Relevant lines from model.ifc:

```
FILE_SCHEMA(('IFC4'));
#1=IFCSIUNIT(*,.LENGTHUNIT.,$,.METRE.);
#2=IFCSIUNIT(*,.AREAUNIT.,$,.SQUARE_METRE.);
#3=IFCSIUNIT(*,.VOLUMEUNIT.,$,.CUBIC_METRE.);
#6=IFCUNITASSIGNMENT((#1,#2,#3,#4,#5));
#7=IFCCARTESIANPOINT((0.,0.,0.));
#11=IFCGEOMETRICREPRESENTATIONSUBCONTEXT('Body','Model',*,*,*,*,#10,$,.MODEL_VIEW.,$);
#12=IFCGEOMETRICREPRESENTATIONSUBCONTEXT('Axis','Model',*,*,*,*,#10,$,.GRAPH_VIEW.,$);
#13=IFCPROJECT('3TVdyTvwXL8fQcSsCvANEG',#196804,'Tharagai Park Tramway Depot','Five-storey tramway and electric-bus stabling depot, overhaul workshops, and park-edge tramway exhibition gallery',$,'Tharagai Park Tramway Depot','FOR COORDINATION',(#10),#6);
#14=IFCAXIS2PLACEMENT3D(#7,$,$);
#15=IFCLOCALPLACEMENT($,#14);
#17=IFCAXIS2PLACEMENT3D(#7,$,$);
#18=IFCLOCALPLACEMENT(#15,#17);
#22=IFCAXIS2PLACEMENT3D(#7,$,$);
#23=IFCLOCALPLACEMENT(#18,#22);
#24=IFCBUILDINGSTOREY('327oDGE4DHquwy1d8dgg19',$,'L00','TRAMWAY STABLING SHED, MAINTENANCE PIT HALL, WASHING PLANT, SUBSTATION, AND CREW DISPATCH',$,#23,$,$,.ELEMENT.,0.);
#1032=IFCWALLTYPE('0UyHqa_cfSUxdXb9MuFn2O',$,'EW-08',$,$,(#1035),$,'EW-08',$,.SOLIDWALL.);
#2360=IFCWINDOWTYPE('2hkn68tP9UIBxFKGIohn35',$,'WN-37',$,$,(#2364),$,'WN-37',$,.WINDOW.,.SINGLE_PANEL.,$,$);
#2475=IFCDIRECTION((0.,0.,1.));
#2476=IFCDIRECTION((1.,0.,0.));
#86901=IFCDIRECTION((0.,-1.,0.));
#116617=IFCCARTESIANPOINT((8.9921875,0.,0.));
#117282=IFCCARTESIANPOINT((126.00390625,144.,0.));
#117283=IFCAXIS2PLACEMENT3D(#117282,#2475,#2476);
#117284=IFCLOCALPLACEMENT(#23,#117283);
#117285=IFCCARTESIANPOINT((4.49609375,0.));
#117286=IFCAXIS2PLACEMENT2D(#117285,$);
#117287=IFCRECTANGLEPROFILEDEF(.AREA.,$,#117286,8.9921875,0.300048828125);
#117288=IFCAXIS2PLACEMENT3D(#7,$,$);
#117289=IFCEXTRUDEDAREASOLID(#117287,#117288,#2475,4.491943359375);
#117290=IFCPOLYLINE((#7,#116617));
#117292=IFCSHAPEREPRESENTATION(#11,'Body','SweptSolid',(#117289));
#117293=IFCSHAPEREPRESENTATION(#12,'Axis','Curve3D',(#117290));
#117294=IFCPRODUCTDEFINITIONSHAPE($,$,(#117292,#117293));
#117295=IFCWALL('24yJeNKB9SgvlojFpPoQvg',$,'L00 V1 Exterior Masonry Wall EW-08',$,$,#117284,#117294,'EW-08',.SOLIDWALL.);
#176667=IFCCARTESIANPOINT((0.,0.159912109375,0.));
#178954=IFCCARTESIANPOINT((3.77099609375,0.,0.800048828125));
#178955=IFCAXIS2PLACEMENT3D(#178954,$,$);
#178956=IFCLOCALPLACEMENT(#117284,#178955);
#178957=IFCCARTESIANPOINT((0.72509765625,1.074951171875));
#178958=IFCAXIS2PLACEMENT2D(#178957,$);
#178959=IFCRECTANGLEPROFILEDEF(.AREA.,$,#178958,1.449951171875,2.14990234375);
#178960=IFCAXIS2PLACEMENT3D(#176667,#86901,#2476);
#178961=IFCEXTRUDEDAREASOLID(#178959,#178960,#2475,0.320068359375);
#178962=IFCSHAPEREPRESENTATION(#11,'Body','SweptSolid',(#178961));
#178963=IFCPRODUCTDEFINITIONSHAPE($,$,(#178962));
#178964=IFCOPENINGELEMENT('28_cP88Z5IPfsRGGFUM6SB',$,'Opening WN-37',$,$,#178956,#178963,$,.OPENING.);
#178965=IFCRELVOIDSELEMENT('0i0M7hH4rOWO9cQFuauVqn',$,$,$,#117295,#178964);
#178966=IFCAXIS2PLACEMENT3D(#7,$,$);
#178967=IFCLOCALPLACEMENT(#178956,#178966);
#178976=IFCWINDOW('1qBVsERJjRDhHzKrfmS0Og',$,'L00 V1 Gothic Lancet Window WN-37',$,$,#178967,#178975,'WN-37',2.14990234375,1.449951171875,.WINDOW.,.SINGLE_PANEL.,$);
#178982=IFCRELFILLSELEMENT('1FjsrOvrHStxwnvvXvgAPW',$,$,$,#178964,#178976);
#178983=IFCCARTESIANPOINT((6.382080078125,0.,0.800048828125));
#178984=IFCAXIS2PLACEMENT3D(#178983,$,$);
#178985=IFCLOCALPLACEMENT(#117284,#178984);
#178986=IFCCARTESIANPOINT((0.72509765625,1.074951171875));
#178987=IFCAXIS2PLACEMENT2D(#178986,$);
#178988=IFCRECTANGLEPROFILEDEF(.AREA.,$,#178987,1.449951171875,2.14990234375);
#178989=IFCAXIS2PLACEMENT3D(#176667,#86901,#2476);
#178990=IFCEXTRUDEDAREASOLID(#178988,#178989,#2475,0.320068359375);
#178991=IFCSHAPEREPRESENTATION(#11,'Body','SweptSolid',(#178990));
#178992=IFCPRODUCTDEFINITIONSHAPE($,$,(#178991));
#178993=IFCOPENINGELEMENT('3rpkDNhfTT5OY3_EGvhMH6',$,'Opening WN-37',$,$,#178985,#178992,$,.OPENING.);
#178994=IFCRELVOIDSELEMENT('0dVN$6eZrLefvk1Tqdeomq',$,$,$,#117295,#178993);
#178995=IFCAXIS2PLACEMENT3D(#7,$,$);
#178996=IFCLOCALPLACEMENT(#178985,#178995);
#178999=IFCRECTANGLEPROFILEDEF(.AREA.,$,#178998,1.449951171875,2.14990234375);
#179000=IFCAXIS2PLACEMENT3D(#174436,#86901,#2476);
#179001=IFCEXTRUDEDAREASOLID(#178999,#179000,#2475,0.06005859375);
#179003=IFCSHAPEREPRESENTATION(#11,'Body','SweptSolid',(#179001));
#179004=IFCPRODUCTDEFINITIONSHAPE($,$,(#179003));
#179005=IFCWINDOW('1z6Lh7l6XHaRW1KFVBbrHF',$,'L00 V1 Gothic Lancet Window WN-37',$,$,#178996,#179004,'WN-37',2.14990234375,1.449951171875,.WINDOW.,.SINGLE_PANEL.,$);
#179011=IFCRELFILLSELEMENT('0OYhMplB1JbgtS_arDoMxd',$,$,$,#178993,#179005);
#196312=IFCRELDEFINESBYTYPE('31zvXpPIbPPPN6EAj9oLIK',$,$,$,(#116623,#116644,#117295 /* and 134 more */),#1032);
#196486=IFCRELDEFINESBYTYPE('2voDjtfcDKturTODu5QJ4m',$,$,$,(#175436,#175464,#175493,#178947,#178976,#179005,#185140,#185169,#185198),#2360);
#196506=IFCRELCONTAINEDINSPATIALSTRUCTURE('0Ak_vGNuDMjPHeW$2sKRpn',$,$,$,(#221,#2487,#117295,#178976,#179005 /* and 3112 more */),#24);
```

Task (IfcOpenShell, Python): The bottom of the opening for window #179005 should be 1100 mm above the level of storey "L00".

```python
import numpy as np
import ifcopenshell
import ifcopenshell.api.geometry
import ifcopenshell.geom
import ifcopenshell.util.element
import ifcopenshell.util.placement
import ifcopenshell.util.shape
import ifcopenshell.util.unit

model = ifcopenshell.open("model.ifc")
unit_scale = ifcopenshell.util.unit.calculate_unit_scale(model)

window = model.by_guid("1z6Lh7l6XHaRW1KFVBbrHF")
opening = window.FillsVoids[0].RelatingOpeningElement
storey = ifcopenshell.util.element.get_container(window, ifc_class="IfcBuildingStorey")
level = ifcopenshell.util.placement.get_local_placement(storey.ObjectPlacement)[2, 3]

# The opening's origin need not be at the sill, so measure its lowest point.
shape = ifcopenshell.geom.create_shape(ifcopenshell.geom.settings(), opening)
bottom = ifcopenshell.util.shape.get_shape_bottom_elevation(shape, shape.geometry) / unit_scale
dz = level + 1.1 / unit_scale - bottom

shift = np.array([0.0, 0.0, dz])
# The window is placed relative to its opening, so it follows when the opening moves.
matrix = ifcopenshell.util.placement.get_local_placement(opening.ObjectPlacement)
matrix[:3, 3] += shift
ifcopenshell.api.geometry.edit_object_placement(
    model, product=opening, matrix=matrix, is_si=False, should_transform_children=True
)

print(f"moved by {dz * unit_scale:+.3f} m")

model.write("model_rev.ifc")
```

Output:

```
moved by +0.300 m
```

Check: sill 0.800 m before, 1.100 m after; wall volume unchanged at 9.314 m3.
